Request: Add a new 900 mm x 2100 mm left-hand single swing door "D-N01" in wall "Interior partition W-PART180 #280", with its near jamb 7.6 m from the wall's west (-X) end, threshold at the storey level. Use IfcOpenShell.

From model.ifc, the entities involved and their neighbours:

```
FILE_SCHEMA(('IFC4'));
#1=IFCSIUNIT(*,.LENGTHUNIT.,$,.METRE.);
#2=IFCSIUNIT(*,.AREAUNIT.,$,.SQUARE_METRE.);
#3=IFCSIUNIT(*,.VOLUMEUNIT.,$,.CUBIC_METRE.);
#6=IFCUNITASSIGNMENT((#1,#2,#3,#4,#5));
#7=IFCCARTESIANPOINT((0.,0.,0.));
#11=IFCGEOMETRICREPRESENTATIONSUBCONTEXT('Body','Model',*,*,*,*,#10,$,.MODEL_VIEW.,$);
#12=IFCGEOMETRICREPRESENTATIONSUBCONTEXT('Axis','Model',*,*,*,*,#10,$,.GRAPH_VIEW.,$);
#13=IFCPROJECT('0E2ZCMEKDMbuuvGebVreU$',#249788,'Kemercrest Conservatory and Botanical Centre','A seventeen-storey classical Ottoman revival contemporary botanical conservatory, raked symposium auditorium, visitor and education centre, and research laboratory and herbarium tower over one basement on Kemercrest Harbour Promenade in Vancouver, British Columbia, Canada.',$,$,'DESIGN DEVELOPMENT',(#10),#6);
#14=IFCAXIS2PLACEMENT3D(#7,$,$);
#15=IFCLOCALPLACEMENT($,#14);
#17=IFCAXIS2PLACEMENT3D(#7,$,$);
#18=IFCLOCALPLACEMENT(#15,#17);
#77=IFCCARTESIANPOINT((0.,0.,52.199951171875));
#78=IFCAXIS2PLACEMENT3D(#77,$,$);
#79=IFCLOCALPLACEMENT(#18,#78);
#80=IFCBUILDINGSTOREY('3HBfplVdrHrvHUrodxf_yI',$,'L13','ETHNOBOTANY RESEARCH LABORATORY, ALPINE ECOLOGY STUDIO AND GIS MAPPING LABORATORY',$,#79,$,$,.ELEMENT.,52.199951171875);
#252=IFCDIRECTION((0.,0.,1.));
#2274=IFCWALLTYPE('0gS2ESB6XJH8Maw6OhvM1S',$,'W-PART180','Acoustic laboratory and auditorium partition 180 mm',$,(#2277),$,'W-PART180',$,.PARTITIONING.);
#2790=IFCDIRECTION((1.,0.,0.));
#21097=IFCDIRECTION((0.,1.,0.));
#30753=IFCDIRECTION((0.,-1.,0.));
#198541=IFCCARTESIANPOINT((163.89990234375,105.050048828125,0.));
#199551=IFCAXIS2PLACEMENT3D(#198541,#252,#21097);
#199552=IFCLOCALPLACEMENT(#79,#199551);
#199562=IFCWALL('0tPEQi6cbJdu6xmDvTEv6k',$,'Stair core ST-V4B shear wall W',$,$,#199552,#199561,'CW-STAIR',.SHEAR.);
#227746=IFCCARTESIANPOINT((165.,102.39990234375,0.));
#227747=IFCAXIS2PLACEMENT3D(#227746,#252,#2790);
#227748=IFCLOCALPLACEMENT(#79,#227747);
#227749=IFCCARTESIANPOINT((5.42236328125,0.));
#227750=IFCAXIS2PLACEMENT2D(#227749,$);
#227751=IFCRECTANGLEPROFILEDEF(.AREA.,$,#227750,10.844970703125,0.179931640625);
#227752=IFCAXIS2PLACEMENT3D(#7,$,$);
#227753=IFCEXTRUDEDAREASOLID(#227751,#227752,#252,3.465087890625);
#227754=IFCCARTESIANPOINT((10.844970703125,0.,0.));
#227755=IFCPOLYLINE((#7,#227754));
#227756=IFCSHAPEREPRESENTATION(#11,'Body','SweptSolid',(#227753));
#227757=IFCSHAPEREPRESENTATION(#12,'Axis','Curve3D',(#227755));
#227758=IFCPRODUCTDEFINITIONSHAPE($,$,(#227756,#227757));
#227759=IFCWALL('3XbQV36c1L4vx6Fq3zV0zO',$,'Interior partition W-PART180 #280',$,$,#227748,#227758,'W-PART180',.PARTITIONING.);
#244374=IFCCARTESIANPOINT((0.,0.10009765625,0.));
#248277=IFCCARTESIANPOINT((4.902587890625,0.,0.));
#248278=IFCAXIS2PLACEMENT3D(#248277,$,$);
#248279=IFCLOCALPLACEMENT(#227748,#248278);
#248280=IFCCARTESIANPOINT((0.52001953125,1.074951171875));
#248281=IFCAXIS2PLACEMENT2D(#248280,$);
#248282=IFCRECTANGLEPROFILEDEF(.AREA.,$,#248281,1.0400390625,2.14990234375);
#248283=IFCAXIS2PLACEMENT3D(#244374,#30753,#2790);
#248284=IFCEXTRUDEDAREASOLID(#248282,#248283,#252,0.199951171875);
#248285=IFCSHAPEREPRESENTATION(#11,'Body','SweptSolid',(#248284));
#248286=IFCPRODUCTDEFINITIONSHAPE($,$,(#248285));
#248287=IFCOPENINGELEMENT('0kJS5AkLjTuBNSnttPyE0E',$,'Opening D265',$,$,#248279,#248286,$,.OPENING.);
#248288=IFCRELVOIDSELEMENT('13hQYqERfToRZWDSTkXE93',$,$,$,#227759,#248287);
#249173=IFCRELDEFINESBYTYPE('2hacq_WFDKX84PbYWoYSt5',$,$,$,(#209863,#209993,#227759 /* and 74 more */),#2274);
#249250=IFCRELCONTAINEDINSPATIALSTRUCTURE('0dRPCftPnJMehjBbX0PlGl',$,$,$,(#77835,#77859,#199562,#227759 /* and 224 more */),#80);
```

```python
import numpy as np
import ifcopenshell
import ifcopenshell.api.feature
import ifcopenshell.api.geometry
import ifcopenshell.api.root
import ifcopenshell.api.spatial
import ifcopenshell.geom
import ifcopenshell.util.element
import ifcopenshell.util.placement
import ifcopenshell.util.representation
import ifcopenshell.util.shape
import ifcopenshell.util.unit

model = ifcopenshell.open("model.ifc")
unit_scale = ifcopenshell.util.unit.calculate_unit_scale(model)
settings = ifcopenshell.geom.settings()


def volume(element):
    """Net volume in cubic metres, openings subtracted."""
    shape = ifcopenshell.geom.create_shape(settings, element)
    return ifcopenshell.util.shape.get_volume(shape.geometry)


wall = model.by_guid("3XbQV36c1L4vx6Fq3zV0zO")
storey = ifcopenshell.util.element.get_container(wall, ifc_class="IfcBuildingStorey")
context = ifcopenshell.util.representation.get_context(model, "Model", "Body", "MODEL_VIEW")
before = volume(wall)

width, height, from_end, sill = 0.9, 2.1, 7.6, 0.0  # metres

# The wall runs along its own X axis, and the end named is its -X end.
wall_shape = ifcopenshell.geom.create_shape(settings, wall)
x, y, z = ifcopenshell.util.shape.get_vertices(wall_shape.geometry).T
start = x.min() + from_end
face, thickness = float(y.min()), float(y.max() - y.min())
wall_matrix = ifcopenshell.util.placement.get_local_placement(wall.ObjectPlacement)
level = ifcopenshell.util.placement.get_local_placement(storey.ObjectPlacement)[2, 3]


def in_wall(x, y):
    """Placement at x, y metres in the wall's axes, at sill height."""
    matrix = wall_matrix.copy()
    matrix[:, 3] = wall_matrix @ np.array([x / unit_scale, y / unit_scale, 0.0, 1.0])
    matrix[2, 3] = level + sill / unit_scale
    return matrix


# Opening: a box that overshoots both wall faces by 50 mm.
opening = ifcopenshell.api.root.create_entity(model, ifc_class="IfcOpeningElement", predefined_type="OPENING")
box = ifcopenshell.api.geometry.add_wall_representation(
    model, context=context, length=width, height=height, thickness=thickness + 0.1
)
ifcopenshell.api.geometry.assign_representation(model, product=opening, representation=box)
ifcopenshell.api.geometry.edit_object_placement(model, product=opening, matrix=in_wall(start, face - 0.05), is_si=False)
ifcopenshell.api.feature.add_feature(model, feature=opening, element=wall)

door = ifcopenshell.api.root.create_entity(model, ifc_class="IfcDoor", name="D-N01", predefined_type="DOOR")
door.OverallWidth, door.OverallHeight = width / unit_scale, height / unit_scale
door.OperationType = "SINGLE_SWING_LEFT"
body = ifcopenshell.api.geometry.add_door_representation(
    model,
    context=context,
    overall_width=door.OverallWidth,
    overall_height=door.OverallHeight,
    operation_type="SINGLE_SWING_LEFT",
    lining_properties={"LiningDepth": thickness / unit_scale, "ThresholdDepth": thickness / unit_scale},
)
ifcopenshell.api.geometry.assign_representation(model, product=door, representation=body)
ifcopenshell.api.spatial.assign_container(model, products=[door], relating_structure=storey)
ifcopenshell.api.feature.add_filling(model, opening=opening, element=door)

# The lining spans the wall, so the door starts at the wall face.
ifcopenshell.api.geometry.edit_object_placement(model, product=door, matrix=in_wall(start, face), is_si=False)

after = volume(wall)

print(f"wall volume {before:.3f} -> {after:.3f} m3")

model.write("model-out.ifc")
```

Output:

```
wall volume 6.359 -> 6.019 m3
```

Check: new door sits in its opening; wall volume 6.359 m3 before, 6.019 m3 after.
